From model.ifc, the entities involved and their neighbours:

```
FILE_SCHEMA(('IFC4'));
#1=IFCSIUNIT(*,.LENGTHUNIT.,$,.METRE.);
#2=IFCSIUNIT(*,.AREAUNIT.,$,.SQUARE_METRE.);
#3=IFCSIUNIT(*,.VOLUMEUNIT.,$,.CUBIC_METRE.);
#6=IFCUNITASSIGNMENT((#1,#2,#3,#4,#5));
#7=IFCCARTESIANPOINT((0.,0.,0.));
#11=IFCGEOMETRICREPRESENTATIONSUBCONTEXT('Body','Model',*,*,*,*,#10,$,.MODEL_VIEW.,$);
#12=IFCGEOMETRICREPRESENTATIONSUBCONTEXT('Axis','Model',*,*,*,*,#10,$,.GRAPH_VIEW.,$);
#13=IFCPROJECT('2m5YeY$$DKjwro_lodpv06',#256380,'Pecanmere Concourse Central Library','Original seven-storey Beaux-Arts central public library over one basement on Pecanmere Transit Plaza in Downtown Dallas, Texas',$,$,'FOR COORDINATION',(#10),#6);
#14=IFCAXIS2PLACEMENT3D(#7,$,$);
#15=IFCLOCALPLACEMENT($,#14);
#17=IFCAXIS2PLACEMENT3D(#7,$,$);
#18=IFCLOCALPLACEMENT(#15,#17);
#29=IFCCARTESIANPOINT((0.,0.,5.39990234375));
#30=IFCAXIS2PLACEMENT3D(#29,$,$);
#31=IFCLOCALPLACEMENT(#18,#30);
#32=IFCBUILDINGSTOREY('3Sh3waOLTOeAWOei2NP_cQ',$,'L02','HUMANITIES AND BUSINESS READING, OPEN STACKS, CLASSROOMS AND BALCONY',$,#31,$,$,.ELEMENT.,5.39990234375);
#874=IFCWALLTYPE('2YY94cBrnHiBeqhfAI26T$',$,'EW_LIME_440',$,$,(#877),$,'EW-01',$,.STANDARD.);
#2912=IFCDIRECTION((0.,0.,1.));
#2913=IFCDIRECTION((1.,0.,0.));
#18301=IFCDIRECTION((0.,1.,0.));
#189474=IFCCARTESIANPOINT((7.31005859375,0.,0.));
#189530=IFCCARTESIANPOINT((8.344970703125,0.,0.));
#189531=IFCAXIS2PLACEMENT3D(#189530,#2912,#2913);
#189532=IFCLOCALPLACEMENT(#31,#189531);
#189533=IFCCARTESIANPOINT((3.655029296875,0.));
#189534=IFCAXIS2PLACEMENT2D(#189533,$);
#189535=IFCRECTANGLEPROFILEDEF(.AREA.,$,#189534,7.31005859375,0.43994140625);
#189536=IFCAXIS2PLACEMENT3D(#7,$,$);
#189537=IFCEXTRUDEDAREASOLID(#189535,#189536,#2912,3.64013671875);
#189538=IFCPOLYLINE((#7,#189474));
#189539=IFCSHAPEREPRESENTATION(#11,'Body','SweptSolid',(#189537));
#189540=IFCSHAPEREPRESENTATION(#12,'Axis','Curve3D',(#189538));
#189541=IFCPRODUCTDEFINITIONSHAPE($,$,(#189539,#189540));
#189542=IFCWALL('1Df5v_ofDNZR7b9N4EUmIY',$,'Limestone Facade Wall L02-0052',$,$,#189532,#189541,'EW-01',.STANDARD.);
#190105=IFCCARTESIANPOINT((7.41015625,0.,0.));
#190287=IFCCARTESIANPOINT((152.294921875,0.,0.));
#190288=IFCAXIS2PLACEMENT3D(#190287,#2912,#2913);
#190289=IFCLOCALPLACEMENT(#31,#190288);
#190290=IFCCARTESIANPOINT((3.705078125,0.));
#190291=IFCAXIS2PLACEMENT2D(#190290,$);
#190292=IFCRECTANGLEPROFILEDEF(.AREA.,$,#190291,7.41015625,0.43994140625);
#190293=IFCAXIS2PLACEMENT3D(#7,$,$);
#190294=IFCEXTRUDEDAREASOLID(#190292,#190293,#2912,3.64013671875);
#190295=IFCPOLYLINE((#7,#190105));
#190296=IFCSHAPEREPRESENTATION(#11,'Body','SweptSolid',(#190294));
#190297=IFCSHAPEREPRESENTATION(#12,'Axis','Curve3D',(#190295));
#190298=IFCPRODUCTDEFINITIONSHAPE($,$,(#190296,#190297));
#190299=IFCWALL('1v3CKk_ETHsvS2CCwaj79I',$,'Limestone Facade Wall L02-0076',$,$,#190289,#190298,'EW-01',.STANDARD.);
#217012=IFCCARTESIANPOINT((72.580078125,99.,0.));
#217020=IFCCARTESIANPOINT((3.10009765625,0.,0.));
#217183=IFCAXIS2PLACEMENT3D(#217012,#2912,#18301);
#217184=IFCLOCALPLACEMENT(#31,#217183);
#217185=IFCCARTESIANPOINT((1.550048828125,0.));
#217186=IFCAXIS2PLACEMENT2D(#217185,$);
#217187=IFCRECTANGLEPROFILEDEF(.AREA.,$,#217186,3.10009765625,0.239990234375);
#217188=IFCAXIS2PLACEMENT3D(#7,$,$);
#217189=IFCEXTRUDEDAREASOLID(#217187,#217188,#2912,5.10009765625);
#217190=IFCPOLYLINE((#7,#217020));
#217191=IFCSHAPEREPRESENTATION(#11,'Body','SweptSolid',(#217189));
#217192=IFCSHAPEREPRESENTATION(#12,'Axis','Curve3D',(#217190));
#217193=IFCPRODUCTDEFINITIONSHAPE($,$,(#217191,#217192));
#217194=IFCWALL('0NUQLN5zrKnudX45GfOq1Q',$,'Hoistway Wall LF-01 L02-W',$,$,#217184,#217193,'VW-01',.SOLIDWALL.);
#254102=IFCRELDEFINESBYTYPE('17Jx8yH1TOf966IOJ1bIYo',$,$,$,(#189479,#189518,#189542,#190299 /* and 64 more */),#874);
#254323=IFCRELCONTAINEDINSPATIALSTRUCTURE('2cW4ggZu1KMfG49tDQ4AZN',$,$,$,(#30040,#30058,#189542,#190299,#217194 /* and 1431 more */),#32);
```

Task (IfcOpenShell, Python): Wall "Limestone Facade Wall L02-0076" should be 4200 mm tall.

```python
import ifcopenshell
import ifcopenshell.geom
import ifcopenshell.util.representation
import ifcopenshell.util.shape
import ifcopenshell.util.unit

model = ifcopenshell.open("model.ifc")
unit_scale = ifcopenshell.util.unit.calculate_unit_scale(model)
settings = ifcopenshell.geom.settings()


def volume(element):
    """Net volume in cubic metres, openings subtracted."""
    shape = ifcopenshell.geom.create_shape(settings, element)
    return ifcopenshell.util.shape.get_volume(shape.geometry)


wall = model.by_guid("1v3CKk_ETHsvS2CCwaj79I")
before = volume(wall)

body = ifcopenshell.util.representation.get_representation(wall, "Model", "Body")
solid = body.Items[0]
old_height = solid.Depth
solid.Depth = 4.2 / unit_scale
after = volume(wall)

print(f"height {old_height:g} -> {solid.Depth:g}, volume {before:.3f} -> {after:.3f} m3")

model.write("model_updated.ifc")
```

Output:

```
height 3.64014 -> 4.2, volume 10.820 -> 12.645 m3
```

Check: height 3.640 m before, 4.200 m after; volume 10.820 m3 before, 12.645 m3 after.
